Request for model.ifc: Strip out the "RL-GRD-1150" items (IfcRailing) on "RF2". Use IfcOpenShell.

First a look at what the model holds.

```python
import ifcopenshell
import ifcopenshell.util.element

model = ifcopenshell.open("model.ifc")
print(model.schema)
storey = next(s for s in model.by_type("IfcBuildingStorey") if s.Name == "RF2")
railings = [e for e in ifcopenshell.util.element.get_decomposition(storey) if e.is_a("IfcRailing")]
seen = {}
for e in railings:
    element_type = ifcopenshell.util.element.get_type(e)
    name = element_type.Name if element_type not in (None, e) else None
    seen[name] = seen.get(name, 0) + 1
for name, count in sorted(seen.items(), key=str):
    print(count, "x", name)
```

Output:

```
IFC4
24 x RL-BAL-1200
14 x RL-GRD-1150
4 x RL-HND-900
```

```python
import ifcopenshell
import ifcopenshell.api.root
import ifcopenshell.util.element

model = ifcopenshell.open("model.ifc")

storey = next(s for s in model.by_type("IfcBuildingStorey") if s.Name == "RF2")
railings = [e for e in ifcopenshell.util.element.get_decomposition(storey) if e.is_a("IfcRailing")]
targets = [e for e in railings if (t := ifcopenshell.util.element.get_type(e)) not in (None, e) and t.Name == "RL-GRD-1150"]

for e in targets:
    ifcopenshell.api.root.remove_product(model, product=e)
print(len(targets), "removed")

model.write("model_v2.ifc")
```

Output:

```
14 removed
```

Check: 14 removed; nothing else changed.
